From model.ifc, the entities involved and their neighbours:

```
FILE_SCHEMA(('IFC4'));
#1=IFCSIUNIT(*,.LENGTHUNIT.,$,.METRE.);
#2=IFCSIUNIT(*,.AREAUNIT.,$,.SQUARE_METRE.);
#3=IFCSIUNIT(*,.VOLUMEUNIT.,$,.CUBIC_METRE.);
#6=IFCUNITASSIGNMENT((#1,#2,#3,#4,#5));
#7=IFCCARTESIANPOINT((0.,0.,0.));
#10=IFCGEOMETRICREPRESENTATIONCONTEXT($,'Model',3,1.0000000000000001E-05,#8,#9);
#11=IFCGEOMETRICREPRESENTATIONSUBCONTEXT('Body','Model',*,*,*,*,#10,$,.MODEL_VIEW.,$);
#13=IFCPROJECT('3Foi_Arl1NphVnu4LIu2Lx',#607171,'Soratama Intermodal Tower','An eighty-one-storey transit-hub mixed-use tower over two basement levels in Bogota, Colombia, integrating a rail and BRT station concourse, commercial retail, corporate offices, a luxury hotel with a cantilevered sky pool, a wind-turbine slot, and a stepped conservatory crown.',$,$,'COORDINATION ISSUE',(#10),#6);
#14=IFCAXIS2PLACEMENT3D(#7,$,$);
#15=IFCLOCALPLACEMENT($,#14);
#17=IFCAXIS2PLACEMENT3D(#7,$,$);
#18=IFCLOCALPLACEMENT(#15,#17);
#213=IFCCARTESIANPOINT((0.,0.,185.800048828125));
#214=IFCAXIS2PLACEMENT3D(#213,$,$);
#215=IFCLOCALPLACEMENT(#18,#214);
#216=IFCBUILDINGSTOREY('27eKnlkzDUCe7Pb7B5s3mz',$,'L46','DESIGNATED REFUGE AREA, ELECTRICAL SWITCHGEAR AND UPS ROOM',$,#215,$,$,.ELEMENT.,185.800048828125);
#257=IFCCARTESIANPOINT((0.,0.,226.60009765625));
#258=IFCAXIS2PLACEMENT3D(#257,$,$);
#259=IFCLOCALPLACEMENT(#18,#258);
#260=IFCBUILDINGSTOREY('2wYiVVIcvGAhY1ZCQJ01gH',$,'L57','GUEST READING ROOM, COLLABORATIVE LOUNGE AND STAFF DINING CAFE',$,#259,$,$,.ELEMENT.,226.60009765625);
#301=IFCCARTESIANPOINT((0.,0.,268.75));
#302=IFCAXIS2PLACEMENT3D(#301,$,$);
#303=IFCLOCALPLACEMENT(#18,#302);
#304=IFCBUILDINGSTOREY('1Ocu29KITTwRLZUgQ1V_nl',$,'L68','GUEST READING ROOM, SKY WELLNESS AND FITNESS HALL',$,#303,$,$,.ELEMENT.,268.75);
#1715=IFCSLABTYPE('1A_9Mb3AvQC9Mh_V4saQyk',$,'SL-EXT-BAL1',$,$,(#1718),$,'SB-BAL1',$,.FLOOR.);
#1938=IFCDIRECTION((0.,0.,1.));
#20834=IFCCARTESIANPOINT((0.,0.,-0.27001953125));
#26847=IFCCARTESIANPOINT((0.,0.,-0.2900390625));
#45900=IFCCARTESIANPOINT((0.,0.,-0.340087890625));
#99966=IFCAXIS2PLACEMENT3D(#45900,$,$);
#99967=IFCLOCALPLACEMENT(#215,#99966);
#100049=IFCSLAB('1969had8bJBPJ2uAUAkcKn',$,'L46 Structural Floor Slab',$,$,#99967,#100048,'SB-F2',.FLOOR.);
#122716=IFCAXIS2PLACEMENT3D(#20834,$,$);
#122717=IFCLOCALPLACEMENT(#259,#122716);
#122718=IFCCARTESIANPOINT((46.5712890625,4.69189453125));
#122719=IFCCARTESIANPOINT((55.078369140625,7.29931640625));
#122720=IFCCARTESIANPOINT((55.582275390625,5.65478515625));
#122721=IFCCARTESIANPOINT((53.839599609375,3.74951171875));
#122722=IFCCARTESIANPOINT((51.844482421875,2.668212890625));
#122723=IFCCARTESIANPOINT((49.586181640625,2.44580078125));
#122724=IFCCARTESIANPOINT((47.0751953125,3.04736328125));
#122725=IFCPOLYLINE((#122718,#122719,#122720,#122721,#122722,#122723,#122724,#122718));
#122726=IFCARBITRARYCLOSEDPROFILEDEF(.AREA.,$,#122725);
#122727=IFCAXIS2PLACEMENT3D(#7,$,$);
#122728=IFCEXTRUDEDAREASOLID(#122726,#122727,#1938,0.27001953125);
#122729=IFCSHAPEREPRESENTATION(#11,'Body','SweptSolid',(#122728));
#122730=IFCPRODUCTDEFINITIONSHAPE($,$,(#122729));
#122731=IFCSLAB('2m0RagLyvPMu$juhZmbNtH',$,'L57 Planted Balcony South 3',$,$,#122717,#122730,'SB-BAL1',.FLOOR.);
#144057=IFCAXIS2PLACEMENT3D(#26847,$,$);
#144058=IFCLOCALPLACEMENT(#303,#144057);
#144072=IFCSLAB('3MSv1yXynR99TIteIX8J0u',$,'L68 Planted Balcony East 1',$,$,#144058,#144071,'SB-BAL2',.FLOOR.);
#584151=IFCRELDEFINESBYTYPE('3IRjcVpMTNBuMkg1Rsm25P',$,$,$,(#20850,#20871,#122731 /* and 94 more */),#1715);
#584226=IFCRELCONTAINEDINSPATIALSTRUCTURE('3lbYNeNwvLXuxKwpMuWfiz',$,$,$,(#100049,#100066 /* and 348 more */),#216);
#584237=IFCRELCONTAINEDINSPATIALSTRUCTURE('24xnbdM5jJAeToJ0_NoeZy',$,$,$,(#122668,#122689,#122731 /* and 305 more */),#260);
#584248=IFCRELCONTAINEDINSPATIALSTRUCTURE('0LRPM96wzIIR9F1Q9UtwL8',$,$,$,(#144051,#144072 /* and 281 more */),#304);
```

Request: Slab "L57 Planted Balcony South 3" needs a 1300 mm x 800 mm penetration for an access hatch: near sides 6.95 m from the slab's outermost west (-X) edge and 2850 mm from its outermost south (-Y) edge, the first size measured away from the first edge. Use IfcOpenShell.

```python
import numpy as np
import ifcopenshell
import ifcopenshell.api.feature
import ifcopenshell.api.geometry
import ifcopenshell.api.root
import ifcopenshell.geom
import ifcopenshell.util.placement
import ifcopenshell.util.representation
import ifcopenshell.util.shape
import ifcopenshell.util.unit

model = ifcopenshell.open("model.ifc")
unit_scale = ifcopenshell.util.unit.calculate_unit_scale(model)
settings = ifcopenshell.geom.settings()


def volume(element):
    """Net volume in cubic metres, openings subtracted."""
    shape = ifcopenshell.geom.create_shape(settings, element)
    return ifcopenshell.util.shape.get_volume(shape.geometry)


slab = model.by_id(122731)
before = volume(slab)

# Extent in the slab's own axes, in metres. The edges named are its -X and -Y sides.
slab_shape = ifcopenshell.geom.create_shape(settings, slab)
vertices = ifcopenshell.util.shape.get_vertices(slab_shape.geometry)
x_min, y_min, bottom = vertices.min(axis=0)
top = vertices[:, 2].max()

opening = ifcopenshell.api.root.create_entity(model, ifc_class="IfcOpeningElement", name="Access hatch opening", predefined_type="OPENING")
context = ifcopenshell.util.representation.get_context(model, "Model", "Body", "MODEL_VIEW")
width, depth = 1.3, 0.8
outline = [(0.0, 0.0), (width, 0.0), (width, depth), (0.0, depth), (0.0, 0.0)]
# Overshoot both faces by 50 mm so the cut is clean.
shape = ifcopenshell.api.geometry.add_slab_representation(
    model, context=context, depth=top - bottom + 0.1, polyline=outline
)
ifcopenshell.api.geometry.assign_representation(model, product=opening, representation=shape)

matrix = ifcopenshell.util.placement.get_local_placement(slab.ObjectPlacement)
matrix[:, 3] = matrix @ np.append(np.array([x_min + 6.95, y_min + 2.85, bottom - 0.05]) / unit_scale, 1.0)
ifcopenshell.api.geometry.edit_object_placement(model, product=opening, matrix=matrix, is_si=False)
ifcopenshell.api.feature.add_feature(model, feature=opening, element=slab)

after = volume(slab)

print(f"slab volume {before:.3f} -> {after:.3f} m3")

model.write("model_edited.ifc")
```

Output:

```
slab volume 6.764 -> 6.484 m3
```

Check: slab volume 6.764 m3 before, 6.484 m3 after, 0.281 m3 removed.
